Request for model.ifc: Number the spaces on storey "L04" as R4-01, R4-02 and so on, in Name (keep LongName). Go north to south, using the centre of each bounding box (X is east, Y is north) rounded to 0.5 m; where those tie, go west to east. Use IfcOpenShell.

First a look at what the model holds.

```python
import ifcopenshell
import ifcopenshell.util.element
import ifcopenshell.util.placement

model = ifcopenshell.open("model.ifc")
print(model.schema)
storey = next(s for s in model.by_type("IfcBuildingStorey") if s.Name == "L04")
spaces = [e for e in ifcopenshell.util.element.get_decomposition(storey) if e.is_a("IfcSpace")]
for e in sorted(spaces, key=lambda e: e.id()):
    origin = ifcopenshell.util.placement.get_local_placement(e.ObjectPlacement)[:3, 3]
    print(e.id(), e.Name, e.LongName, origin.round(2) + 0.0, sep=" | ")
```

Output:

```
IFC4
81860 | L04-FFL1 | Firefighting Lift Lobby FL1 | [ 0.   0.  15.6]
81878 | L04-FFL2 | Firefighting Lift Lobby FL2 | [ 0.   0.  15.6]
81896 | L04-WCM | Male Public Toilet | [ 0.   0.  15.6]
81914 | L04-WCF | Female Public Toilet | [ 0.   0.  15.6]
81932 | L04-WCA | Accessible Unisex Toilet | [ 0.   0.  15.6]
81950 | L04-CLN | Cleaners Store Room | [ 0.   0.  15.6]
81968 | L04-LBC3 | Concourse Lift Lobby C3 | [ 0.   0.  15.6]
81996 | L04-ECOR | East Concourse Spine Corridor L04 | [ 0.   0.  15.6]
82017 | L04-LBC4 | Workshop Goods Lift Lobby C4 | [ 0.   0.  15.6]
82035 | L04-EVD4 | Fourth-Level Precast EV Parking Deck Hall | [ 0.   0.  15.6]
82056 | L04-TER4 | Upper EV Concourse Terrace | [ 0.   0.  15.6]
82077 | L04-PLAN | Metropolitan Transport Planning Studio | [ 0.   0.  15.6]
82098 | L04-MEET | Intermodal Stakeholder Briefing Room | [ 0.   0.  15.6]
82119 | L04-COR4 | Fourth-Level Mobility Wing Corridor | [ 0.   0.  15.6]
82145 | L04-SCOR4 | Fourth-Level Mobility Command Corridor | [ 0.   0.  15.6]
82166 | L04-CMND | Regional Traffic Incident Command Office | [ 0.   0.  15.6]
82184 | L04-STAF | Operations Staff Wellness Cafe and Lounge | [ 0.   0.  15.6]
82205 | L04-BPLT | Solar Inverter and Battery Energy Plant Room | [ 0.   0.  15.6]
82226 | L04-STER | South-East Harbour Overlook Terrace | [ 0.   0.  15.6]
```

```python
import ifcopenshell
import ifcopenshell.geom
import ifcopenshell.util.element
import ifcopenshell.util.shape

model = ifcopenshell.open("model.ifc")
settings = ifcopenshell.geom.settings()
settings.set("use-world-coords", True)


def centre(element):
    shape = ifcopenshell.geom.create_shape(settings, element)
    return ifcopenshell.util.shape.get_bbox_centroid(shape.geometry)


storey = next(s for s in model.by_type("IfcBuildingStorey") if s.Name == "L04")
spaces = [e for e in ifcopenshell.util.element.get_decomposition(storey) if e.is_a("IfcSpace")]

# Insertion points can sit at a corner or the storey origin, so sort by the geometry (in metres).
centres = {e: centre(e) for e in spaces}
spaces.sort(key=lambda e: (-round(centres[e][1] / 0.5), centres[e][0]))

for i, e in enumerate(spaces, start=1):
    number = f"R4-{i:02d}"
    e.Name = number
    print(e.id(), number)

model.write("model_rev.ifc")
```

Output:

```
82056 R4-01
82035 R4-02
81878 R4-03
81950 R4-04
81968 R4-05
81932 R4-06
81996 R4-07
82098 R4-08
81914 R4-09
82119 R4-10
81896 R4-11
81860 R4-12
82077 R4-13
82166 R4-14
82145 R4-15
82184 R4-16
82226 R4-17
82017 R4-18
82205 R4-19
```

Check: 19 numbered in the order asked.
